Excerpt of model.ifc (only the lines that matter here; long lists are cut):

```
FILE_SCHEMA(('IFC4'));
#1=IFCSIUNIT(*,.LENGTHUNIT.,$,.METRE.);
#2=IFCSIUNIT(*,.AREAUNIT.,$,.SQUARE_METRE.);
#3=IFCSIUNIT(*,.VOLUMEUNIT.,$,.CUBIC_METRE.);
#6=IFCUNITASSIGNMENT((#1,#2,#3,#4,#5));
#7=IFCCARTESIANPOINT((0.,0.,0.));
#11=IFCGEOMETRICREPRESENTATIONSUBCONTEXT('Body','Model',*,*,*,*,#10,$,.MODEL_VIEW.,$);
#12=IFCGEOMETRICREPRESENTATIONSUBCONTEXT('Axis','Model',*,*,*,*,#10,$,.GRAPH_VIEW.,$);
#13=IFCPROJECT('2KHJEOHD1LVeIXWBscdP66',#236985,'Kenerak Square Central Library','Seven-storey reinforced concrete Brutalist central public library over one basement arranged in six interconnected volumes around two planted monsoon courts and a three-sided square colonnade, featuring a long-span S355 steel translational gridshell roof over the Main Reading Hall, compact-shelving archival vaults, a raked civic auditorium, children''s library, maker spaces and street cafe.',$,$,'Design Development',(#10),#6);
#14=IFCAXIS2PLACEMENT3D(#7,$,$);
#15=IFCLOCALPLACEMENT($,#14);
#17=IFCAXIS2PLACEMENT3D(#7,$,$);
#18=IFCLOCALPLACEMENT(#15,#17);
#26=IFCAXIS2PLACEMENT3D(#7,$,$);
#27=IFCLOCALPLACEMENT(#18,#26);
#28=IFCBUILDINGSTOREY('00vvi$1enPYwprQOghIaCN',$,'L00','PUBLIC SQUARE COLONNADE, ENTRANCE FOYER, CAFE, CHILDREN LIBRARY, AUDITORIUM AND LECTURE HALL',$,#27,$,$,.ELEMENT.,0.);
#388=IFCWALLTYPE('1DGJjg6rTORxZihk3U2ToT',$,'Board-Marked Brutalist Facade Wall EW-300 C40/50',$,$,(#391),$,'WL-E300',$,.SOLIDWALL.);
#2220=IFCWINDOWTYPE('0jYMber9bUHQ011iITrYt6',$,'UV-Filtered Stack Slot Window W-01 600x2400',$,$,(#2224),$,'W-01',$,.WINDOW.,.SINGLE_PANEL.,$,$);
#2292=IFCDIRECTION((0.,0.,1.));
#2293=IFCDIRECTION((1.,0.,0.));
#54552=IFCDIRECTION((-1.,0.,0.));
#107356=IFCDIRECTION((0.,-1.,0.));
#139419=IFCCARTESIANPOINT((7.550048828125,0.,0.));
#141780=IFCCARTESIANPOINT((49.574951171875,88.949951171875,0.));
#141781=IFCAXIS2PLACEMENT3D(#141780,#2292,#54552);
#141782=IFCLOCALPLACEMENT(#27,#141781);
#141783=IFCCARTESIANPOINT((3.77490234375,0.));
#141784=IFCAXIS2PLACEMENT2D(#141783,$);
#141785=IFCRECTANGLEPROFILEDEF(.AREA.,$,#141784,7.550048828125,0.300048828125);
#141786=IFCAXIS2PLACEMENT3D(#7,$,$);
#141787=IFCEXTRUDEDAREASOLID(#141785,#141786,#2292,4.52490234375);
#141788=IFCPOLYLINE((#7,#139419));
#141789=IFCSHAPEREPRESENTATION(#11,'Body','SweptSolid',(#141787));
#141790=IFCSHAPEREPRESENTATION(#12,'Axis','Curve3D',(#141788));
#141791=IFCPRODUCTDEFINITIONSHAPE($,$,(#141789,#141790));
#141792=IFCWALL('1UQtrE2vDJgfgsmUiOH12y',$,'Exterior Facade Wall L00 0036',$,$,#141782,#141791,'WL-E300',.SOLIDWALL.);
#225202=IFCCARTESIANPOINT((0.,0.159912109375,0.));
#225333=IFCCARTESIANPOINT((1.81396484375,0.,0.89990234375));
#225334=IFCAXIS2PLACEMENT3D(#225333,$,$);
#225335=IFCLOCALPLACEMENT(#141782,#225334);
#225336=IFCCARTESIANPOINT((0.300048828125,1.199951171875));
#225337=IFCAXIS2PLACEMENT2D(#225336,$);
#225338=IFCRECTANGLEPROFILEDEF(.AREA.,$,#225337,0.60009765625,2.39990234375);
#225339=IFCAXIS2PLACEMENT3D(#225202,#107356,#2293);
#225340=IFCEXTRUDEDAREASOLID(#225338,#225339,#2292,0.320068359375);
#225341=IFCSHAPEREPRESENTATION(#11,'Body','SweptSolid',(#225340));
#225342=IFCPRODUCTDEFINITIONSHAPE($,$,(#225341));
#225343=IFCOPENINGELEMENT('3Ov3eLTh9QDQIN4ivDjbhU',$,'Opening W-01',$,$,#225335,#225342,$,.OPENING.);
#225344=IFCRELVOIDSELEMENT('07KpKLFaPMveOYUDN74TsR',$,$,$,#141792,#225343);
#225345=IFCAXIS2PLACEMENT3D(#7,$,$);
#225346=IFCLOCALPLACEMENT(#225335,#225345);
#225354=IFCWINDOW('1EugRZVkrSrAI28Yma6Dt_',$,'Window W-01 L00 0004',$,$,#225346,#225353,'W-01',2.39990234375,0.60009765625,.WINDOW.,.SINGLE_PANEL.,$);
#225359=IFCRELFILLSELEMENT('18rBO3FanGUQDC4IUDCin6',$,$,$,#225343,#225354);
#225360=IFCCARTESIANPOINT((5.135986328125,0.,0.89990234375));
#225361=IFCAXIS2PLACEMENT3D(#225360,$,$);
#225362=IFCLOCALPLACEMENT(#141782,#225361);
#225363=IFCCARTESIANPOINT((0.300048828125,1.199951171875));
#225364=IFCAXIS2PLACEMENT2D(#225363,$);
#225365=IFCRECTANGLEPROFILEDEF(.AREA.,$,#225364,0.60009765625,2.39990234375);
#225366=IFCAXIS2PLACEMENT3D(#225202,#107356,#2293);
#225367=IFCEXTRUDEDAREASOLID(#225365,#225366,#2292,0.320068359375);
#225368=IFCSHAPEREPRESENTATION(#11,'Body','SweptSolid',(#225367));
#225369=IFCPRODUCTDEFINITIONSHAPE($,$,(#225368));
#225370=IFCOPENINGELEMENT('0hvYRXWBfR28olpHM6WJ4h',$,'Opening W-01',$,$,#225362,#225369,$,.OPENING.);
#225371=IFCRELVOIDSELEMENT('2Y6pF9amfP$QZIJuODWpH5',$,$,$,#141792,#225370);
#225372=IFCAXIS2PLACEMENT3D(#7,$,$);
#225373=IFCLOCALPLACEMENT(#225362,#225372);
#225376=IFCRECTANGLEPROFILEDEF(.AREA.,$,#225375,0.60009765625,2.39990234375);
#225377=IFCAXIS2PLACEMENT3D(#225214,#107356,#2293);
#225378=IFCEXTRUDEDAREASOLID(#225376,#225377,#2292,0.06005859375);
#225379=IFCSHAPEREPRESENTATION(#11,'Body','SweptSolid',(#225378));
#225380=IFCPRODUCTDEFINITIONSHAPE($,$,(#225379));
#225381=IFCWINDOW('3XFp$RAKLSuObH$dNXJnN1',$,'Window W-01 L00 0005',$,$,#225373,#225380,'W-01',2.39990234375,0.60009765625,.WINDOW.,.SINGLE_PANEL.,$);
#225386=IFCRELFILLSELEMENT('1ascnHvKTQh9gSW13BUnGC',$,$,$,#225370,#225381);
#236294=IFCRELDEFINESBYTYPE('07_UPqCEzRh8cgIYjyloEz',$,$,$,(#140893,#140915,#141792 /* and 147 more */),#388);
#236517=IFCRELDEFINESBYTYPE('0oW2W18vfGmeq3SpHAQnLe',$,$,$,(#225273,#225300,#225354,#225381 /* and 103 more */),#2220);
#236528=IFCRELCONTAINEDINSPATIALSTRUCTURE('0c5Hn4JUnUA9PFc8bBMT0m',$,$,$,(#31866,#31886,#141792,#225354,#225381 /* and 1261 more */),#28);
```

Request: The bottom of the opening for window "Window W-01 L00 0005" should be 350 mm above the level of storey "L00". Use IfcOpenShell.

```python
import numpy as np
import ifcopenshell
import ifcopenshell.api.geometry
import ifcopenshell.geom
import ifcopenshell.util.element
import ifcopenshell.util.placement
import ifcopenshell.util.shape
import ifcopenshell.util.unit

model = ifcopenshell.open("model.ifc")
unit_scale = ifcopenshell.util.unit.calculate_unit_scale(model)

window = model.by_guid("3XFp$RAKLSuObH$dNXJnN1")
opening = window.FillsVoids[0].RelatingOpeningElement
storey = ifcopenshell.util.element.get_container(window, ifc_class="IfcBuildingStorey")
level = ifcopenshell.util.placement.get_local_placement(storey.ObjectPlacement)[2, 3]

# The opening's origin need not be at the sill, so measure its lowest point.
shape = ifcopenshell.geom.create_shape(ifcopenshell.geom.settings(), opening)
bottom = ifcopenshell.util.shape.get_shape_bottom_elevation(shape, shape.geometry) / unit_scale
dz = level + 0.35 / unit_scale - bottom

shift = np.array([0.0, 0.0, dz])
# The window is placed relative to its opening, so it follows when the opening moves.
matrix = ifcopenshell.util.placement.get_local_placement(opening.ObjectPlacement)
matrix[:3, 3] += shift
ifcopenshell.api.geometry.edit_object_placement(
    model, product=opening, matrix=matrix, is_si=False, should_transform_children=True
)

print(f"moved by {dz * unit_scale:+.3f} m")

model.write("model-out.ifc")
```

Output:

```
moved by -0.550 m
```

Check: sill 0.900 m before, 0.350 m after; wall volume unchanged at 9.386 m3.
